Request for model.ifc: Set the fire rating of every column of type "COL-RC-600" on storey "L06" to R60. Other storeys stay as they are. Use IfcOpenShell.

First a look at what the model holds.

```python
import ifcopenshell
import ifcopenshell.util.element

model = ifcopenshell.open("model.ifc")
print(model.schema)
storey = next(s for s in model.by_type("IfcBuildingStorey") if s.Name == "L06")
columns = [e for e in ifcopenshell.util.element.get_decomposition(storey) if e.is_a("IfcColumn")]
seen = {}
for e in columns:
    element_type = ifcopenshell.util.element.get_type(e)
    key = (element_type.Name if element_type != e and element_type else None, ifcopenshell.util.element.get_pset(e, "Pset_ColumnCommon", "FireRating"))
    seen[key] = seen.get(key, 0) + 1
for (name, value), count in sorted(seen.items(), key=str):
    print(count, "x", name, "|", value)
```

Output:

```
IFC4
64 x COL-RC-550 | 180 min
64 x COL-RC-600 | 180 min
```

```python
import ifcopenshell
import ifcopenshell.api.pset
import ifcopenshell.util.element

model = ifcopenshell.open("model.ifc")

storey = next(s for s in model.by_type("IfcBuildingStorey") if s.Name == "L06")
columns = [e for e in ifcopenshell.util.element.get_decomposition(storey) if e.is_a("IfcColumn")]

count = 0
for e in columns:
    element_type = ifcopenshell.util.element.get_type(e)
    if element_type in (None, e) or element_type.Name != "COL-RC-600":
        continue
    # add_pset returns the element's existing set when there is one.
    pset = ifcopenshell.api.pset.add_pset(model, product=e, name="Pset_ColumnCommon")
    ifcopenshell.api.pset.edit_pset(model, pset=pset, properties={"FireRating": "R60"})
    count += 1

print(count, "columns updated")

model.write("model_updated.ifc")
```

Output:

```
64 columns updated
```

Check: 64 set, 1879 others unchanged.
